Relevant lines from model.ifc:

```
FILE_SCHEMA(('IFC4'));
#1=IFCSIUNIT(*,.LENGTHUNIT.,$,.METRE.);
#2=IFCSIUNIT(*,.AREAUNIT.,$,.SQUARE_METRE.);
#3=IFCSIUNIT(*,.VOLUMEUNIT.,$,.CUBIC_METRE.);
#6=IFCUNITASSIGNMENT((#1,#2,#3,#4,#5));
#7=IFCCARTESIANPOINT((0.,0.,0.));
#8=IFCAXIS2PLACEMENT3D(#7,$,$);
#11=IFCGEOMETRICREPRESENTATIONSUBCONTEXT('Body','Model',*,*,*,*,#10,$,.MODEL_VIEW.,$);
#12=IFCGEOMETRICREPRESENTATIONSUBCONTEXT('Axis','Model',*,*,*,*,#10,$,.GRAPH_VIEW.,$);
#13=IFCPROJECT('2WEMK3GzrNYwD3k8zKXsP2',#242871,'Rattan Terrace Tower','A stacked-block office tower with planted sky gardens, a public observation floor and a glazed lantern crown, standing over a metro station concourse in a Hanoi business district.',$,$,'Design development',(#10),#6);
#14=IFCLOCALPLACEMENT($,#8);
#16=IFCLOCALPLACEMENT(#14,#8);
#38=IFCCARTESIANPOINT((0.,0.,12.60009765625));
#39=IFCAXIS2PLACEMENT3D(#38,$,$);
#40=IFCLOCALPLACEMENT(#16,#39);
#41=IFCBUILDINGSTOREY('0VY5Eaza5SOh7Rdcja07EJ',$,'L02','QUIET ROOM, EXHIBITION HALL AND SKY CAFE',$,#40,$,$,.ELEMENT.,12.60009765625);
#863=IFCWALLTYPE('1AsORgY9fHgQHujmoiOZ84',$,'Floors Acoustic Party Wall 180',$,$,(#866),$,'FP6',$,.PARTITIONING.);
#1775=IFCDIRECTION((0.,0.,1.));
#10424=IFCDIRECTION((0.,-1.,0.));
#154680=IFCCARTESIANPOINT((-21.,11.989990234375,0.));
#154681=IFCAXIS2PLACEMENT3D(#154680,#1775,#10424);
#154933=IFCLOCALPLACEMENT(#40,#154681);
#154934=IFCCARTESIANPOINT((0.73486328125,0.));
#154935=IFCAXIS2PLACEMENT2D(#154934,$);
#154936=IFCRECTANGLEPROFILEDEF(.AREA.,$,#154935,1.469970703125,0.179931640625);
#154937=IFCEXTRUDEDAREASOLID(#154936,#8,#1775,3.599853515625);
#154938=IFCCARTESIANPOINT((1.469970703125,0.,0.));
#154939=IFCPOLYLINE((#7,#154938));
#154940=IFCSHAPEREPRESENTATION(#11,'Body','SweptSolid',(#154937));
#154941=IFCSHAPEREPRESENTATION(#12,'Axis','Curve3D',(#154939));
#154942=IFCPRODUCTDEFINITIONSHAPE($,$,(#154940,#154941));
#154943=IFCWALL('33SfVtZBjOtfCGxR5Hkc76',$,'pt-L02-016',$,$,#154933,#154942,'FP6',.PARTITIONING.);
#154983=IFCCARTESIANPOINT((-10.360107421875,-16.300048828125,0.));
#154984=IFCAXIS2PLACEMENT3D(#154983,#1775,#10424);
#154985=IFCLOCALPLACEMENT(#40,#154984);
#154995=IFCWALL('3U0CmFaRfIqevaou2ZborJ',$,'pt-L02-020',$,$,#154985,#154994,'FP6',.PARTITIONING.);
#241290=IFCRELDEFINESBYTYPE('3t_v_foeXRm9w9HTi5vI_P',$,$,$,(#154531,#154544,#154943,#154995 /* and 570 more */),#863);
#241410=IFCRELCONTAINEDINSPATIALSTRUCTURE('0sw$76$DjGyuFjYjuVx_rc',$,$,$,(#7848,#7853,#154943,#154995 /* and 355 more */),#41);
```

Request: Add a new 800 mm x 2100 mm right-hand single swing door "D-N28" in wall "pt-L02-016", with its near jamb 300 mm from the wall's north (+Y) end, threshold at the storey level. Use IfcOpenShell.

```python
import numpy as np
import ifcopenshell
import ifcopenshell.api.feature
import ifcopenshell.api.geometry
import ifcopenshell.api.root
import ifcopenshell.api.spatial
import ifcopenshell.geom
import ifcopenshell.util.element
import ifcopenshell.util.placement
import ifcopenshell.util.representation
import ifcopenshell.util.shape
import ifcopenshell.util.unit

model = ifcopenshell.open("model.ifc")
unit_scale = ifcopenshell.util.unit.calculate_unit_scale(model)
settings = ifcopenshell.geom.settings()


def volume(element):
    """Net volume in cubic metres, openings subtracted."""
    shape = ifcopenshell.geom.create_shape(settings, element)
    return ifcopenshell.util.shape.get_volume(shape.geometry)


wall = model.by_id(154943)
storey = ifcopenshell.util.element.get_container(wall, ifc_class="IfcBuildingStorey")
context = ifcopenshell.util.representation.get_context(model, "Model", "Body", "MODEL_VIEW")
before = volume(wall)

width, height, from_end, sill = 0.8, 2.1, 0.3, 0.0  # metres

# The wall runs along its own X axis, and the end named is its -X end.
wall_shape = ifcopenshell.geom.create_shape(settings, wall)
x, y, z = ifcopenshell.util.shape.get_vertices(wall_shape.geometry).T
start = x.min() + from_end
face, thickness = float(y.min()), float(y.max() - y.min())
wall_matrix = ifcopenshell.util.placement.get_local_placement(wall.ObjectPlacement)
level = ifcopenshell.util.placement.get_local_placement(storey.ObjectPlacement)[2, 3]


def in_wall(x, y):
    """Placement at x, y metres in the wall's axes, at sill height."""
    matrix = wall_matrix.copy()
    matrix[:, 3] = wall_matrix @ np.array([x / unit_scale, y / unit_scale, 0.0, 1.0])
    matrix[2, 3] = level + sill / unit_scale
    return matrix


# Opening: a box that overshoots both wall faces by 50 mm.
opening = ifcopenshell.api.root.create_entity(model, ifc_class="IfcOpeningElement", predefined_type="OPENING")
box = ifcopenshell.api.geometry.add_wall_representation(
    model, context=context, length=width, height=height, thickness=thickness + 0.1
)
ifcopenshell.api.geometry.assign_representation(model, product=opening, representation=box)
ifcopenshell.api.geometry.edit_object_placement(model, product=opening, matrix=in_wall(start, face - 0.05), is_si=False)
ifcopenshell.api.feature.add_feature(model, feature=opening, element=wall)

door = ifcopenshell.api.root.create_entity(model, ifc_class="IfcDoor", name="D-N28", predefined_type="DOOR")
door.OverallWidth, door.OverallHeight = width / unit_scale, height / unit_scale
door.OperationType = "SINGLE_SWING_RIGHT"
body = ifcopenshell.api.geometry.add_door_representation(
    model,
    context=context,
    overall_width=door.OverallWidth,
    overall_height=door.OverallHeight,
    operation_type="SINGLE_SWING_RIGHT",
    lining_properties={"LiningDepth": thickness / unit_scale, "ThresholdDepth": thickness / unit_scale},
)
ifcopenshell.api.geometry.assign_representation(model, product=door, representation=body)
ifcopenshell.api.spatial.assign_container(model, products=[door], relating_structure=storey)
ifcopenshell.api.feature.add_filling(model, opening=opening, element=door)

# The lining spans the wall, so the door starts at the wall face.
ifcopenshell.api.geometry.edit_object_placement(model, product=door, matrix=in_wall(start, face), is_si=False)

after = volume(wall)

print(f"wall volume {before:.3f} -> {after:.3f} m3")

model.write("model_v2.ifc")
```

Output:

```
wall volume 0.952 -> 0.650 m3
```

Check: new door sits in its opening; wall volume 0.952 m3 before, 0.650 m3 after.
